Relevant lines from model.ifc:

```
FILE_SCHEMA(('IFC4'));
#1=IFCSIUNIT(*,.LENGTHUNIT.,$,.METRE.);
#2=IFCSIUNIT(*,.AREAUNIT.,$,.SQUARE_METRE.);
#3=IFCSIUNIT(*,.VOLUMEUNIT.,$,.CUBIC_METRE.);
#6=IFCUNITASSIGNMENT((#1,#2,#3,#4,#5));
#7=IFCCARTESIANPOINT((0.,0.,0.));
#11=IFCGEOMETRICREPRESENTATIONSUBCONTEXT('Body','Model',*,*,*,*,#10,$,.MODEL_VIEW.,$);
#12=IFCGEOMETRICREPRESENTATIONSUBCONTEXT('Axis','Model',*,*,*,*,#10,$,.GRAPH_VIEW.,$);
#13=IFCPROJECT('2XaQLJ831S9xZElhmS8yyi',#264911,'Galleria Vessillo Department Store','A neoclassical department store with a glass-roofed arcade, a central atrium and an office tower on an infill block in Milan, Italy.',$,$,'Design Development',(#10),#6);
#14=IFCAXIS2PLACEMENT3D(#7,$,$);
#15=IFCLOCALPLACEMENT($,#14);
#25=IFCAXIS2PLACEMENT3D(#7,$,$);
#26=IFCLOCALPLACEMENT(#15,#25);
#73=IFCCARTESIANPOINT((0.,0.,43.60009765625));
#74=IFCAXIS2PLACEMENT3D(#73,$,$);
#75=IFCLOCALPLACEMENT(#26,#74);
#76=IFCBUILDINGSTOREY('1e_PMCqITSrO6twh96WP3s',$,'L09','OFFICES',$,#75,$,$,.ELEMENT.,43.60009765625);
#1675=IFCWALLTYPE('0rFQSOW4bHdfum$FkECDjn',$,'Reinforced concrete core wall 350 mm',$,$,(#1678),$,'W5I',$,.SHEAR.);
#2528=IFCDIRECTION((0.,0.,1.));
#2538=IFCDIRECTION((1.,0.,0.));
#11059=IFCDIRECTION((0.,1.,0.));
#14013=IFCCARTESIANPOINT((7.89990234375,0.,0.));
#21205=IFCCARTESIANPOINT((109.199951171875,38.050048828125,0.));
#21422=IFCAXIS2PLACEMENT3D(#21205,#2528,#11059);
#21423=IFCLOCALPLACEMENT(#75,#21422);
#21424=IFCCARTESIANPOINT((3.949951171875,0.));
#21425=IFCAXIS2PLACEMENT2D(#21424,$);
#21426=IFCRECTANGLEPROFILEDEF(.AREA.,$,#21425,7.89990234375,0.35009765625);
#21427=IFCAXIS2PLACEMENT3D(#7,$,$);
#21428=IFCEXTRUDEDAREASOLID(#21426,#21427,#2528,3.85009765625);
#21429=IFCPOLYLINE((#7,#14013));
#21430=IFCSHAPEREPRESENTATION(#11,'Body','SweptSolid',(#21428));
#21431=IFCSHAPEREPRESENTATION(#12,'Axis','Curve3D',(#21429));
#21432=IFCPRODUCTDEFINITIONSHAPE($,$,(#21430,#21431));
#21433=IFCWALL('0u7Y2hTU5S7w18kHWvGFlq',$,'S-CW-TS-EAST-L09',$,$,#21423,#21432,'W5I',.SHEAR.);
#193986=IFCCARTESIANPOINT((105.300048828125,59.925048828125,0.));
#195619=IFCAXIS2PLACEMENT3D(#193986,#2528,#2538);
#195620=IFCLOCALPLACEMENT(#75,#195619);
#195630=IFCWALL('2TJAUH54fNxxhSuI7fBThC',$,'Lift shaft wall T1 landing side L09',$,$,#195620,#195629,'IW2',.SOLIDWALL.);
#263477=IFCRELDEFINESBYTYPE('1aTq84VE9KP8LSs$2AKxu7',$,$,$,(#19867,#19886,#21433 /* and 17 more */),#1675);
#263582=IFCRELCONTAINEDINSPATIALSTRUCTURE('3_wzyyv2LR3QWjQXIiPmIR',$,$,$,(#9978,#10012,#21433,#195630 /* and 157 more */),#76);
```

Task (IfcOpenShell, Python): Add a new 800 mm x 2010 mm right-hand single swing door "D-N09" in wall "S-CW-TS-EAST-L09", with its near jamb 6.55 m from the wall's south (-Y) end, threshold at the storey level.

```python
import numpy as np
import ifcopenshell
import ifcopenshell.api.feature
import ifcopenshell.api.geometry
import ifcopenshell.api.root
import ifcopenshell.api.spatial
import ifcopenshell.geom
import ifcopenshell.util.element
import ifcopenshell.util.placement
import ifcopenshell.util.representation
import ifcopenshell.util.shape
import ifcopenshell.util.unit

model = ifcopenshell.open("model.ifc")
unit_scale = ifcopenshell.util.unit.calculate_unit_scale(model)
settings = ifcopenshell.geom.settings()


def volume(element):
    """Net volume in cubic metres, openings subtracted."""
    shape = ifcopenshell.geom.create_shape(settings, element)
    return ifcopenshell.util.shape.get_volume(shape.geometry)


wall = model.by_guid("0u7Y2hTU5S7w18kHWvGFlq")
storey = ifcopenshell.util.element.get_container(wall, ifc_class="IfcBuildingStorey")
context = ifcopenshell.util.representation.get_context(model, "Model", "Body", "MODEL_VIEW")
before = volume(wall)

width, height, from_end, sill = 0.8, 2.01, 6.55, 0.0  # metres

# The wall runs along its own X axis, and the end named is its -X end.
wall_shape = ifcopenshell.geom.create_shape(settings, wall)
x, y, z = ifcopenshell.util.shape.get_vertices(wall_shape.geometry).T
start = x.min() + from_end
face, thickness = float(y.min()), float(y.max() - y.min())
wall_matrix = ifcopenshell.util.placement.get_local_placement(wall.ObjectPlacement)
level = ifcopenshell.util.placement.get_local_placement(storey.ObjectPlacement)[2, 3]


def in_wall(x, y):
    """Placement at x, y metres in the wall's axes, at sill height."""
    matrix = wall_matrix.copy()
    matrix[:, 3] = wall_matrix @ np.array([x / unit_scale, y / unit_scale, 0.0, 1.0])
    matrix[2, 3] = level + sill / unit_scale
    return matrix


# Opening: a box that overshoots both wall faces by 50 mm.
opening = ifcopenshell.api.root.create_entity(model, ifc_class="IfcOpeningElement", predefined_type="OPENING")
box = ifcopenshell.api.geometry.add_wall_representation(
    model, context=context, length=width, height=height, thickness=thickness + 0.1
)
ifcopenshell.api.geometry.assign_representation(model, product=opening, representation=box)
ifcopenshell.api.geometry.edit_object_placement(model, product=opening, matrix=in_wall(start, face - 0.05), is_si=False)
ifcopenshell.api.feature.add_feature(model, feature=opening, element=wall)

door = ifcopenshell.api.root.create_entity(model, ifc_class="IfcDoor", name="D-N09", predefined_type="DOOR")
door.OverallWidth, door.OverallHeight = width / unit_scale, height / unit_scale
door.OperationType = "SINGLE_SWING_RIGHT"
body = ifcopenshell.api.geometry.add_door_representation(
    model,
    context=context,
    overall_width=door.OverallWidth,
    overall_height=door.OverallHeight,
    operation_type="SINGLE_SWING_RIGHT",
    lining_properties={"LiningDepth": thickness / unit_scale, "ThresholdDepth": thickness / unit_scale},
)
ifcopenshell.api.geometry.assign_representation(model, product=door, representation=body)
ifcopenshell.api.spatial.assign_container(model, products=[door], relating_structure=storey)
ifcopenshell.api.feature.add_filling(model, opening=opening, element=door)

# The lining spans the wall, so the door starts at the wall face.
ifcopenshell.api.geometry.edit_object_placement(model, product=door, matrix=in_wall(start, face), is_si=False)

after = volume(wall)

print(f"wall volume {before:.3f} -> {after:.3f} m3")

model.write("model_rev.ifc")
```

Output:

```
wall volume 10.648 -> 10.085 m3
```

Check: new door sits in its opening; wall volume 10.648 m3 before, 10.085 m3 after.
